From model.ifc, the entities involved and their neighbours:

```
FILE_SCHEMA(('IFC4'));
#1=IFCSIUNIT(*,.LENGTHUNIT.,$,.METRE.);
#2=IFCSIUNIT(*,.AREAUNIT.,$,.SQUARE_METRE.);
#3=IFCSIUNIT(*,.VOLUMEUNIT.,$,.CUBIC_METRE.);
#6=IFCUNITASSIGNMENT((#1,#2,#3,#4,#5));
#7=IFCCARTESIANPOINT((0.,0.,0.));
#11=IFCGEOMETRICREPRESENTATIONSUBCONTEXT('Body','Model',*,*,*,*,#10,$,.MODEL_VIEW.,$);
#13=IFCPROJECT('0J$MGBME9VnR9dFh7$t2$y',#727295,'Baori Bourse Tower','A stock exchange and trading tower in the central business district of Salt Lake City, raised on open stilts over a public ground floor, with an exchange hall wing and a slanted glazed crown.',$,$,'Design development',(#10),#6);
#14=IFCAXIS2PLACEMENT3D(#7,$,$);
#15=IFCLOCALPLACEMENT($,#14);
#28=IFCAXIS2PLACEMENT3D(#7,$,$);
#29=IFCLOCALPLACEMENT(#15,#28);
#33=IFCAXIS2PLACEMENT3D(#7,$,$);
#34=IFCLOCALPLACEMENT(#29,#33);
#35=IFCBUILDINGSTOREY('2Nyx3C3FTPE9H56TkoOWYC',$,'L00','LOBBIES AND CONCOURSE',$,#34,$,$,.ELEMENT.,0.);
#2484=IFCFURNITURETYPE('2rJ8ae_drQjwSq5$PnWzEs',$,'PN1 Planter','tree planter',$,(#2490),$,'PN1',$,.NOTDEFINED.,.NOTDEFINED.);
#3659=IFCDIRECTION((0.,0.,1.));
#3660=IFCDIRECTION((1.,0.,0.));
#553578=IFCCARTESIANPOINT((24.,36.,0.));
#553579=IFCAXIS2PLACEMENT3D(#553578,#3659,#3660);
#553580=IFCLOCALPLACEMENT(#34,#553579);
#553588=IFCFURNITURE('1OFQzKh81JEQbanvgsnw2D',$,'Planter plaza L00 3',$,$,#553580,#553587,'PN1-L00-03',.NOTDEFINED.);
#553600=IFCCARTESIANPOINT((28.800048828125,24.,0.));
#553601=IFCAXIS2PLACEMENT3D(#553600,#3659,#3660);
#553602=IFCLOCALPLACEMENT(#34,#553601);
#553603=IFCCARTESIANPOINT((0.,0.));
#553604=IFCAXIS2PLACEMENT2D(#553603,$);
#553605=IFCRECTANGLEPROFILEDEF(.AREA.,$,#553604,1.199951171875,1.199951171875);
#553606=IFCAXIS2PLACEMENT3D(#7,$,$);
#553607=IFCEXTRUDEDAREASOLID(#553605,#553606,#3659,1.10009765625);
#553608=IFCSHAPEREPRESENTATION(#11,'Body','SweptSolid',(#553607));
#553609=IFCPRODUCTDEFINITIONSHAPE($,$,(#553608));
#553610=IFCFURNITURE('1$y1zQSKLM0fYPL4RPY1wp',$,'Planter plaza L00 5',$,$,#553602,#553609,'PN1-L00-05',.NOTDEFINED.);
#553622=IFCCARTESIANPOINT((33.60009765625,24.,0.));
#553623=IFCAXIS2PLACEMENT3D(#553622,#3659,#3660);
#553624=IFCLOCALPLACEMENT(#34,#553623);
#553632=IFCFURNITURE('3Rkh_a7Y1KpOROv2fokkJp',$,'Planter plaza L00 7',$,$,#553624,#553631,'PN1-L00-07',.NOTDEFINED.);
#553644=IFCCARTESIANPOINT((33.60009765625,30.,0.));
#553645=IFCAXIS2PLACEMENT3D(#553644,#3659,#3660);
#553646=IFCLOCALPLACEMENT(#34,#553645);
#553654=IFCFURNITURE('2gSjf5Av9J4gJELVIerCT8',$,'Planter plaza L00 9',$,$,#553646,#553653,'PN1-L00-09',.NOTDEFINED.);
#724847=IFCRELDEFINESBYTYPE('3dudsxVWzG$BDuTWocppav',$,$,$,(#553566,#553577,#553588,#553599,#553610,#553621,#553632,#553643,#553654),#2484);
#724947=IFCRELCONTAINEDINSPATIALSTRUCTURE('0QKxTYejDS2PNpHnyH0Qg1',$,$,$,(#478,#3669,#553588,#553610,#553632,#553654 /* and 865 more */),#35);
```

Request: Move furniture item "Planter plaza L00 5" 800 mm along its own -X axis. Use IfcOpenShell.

```python
import ifcopenshell
import ifcopenshell.api.geometry
import ifcopenshell.util.placement

model = ifcopenshell.open("model.ifc")

item = model.by_guid("1$y1zQSKLM0fYPL4RPY1wp")
matrix = ifcopenshell.util.placement.get_local_placement(item.ObjectPlacement)
matrix[:3, 3] -= matrix[:3, 0] * 0.8
ifcopenshell.api.geometry.edit_object_placement(model, product=item, matrix=matrix, is_si=False)

print(ifcopenshell.util.placement.get_local_placement(item.ObjectPlacement).round(3) + 0.0)

model.write("model_v2.ifc")
```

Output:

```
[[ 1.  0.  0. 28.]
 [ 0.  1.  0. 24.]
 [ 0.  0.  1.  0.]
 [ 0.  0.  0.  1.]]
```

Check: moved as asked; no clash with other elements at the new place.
